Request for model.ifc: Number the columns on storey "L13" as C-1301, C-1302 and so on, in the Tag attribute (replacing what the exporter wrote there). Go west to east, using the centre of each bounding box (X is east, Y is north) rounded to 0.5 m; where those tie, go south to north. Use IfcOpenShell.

First a look at what the model holds.

```python
import ifcopenshell
import ifcopenshell.util.element
import ifcopenshell.util.placement

model = ifcopenshell.open("model.ifc")
print(model.schema)
storey = next(s for s in model.by_type("IfcBuildingStorey") if s.Name == "L13")
columns = [e for e in ifcopenshell.util.element.get_decomposition(storey) if e.is_a("IfcColumn")]
for e in sorted(columns, key=lambda e: e.id()):
    origin = ifcopenshell.util.placement.get_local_placement(e.ObjectPlacement)[:3, 3]
    print(e.id(), e.Tag, e.Name, origin.round(2) + 0.0, sep=" | ")
```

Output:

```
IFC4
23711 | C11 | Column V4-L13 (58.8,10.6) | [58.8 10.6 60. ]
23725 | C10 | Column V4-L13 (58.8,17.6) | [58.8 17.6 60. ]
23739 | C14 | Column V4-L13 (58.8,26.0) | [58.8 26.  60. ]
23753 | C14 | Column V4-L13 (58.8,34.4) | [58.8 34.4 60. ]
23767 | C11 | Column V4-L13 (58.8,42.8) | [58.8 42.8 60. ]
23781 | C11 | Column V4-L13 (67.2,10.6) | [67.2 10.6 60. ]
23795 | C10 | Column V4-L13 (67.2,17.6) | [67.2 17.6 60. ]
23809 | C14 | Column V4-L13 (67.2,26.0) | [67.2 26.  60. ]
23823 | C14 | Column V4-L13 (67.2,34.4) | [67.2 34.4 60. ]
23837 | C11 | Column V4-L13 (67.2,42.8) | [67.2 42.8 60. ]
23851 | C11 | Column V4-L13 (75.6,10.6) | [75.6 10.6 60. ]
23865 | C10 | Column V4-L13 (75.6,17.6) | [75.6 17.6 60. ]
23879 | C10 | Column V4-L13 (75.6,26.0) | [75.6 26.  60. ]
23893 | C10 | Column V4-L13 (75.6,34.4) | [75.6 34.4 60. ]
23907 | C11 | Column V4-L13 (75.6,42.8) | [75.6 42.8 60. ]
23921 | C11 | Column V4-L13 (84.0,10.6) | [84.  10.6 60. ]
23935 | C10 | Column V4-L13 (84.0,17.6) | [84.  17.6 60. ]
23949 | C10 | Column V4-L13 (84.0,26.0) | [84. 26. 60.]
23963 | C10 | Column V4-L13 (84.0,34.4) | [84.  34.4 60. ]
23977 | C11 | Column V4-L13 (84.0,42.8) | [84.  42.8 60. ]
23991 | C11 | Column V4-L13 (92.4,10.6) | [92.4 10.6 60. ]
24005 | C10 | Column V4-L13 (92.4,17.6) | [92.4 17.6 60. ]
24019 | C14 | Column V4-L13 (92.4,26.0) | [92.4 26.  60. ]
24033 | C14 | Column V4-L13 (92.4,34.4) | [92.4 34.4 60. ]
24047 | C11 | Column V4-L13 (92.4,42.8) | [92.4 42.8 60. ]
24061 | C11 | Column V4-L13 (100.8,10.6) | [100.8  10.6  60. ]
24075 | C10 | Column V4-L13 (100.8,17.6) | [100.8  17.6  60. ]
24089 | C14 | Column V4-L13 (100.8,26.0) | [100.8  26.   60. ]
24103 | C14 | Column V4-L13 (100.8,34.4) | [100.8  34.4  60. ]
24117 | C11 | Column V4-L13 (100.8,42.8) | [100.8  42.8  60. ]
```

```python
import ifcopenshell
import ifcopenshell.geom
import ifcopenshell.util.element
import ifcopenshell.util.shape

model = ifcopenshell.open("model.ifc")
settings = ifcopenshell.geom.settings()
settings.set("use-world-coords", True)


def centre(element):
    shape = ifcopenshell.geom.create_shape(settings, element)
    return ifcopenshell.util.shape.get_bbox_centroid(shape.geometry)


storey = next(s for s in model.by_type("IfcBuildingStorey") if s.Name == "L13")
columns = [e for e in ifcopenshell.util.element.get_decomposition(storey) if e.is_a("IfcColumn")]

# Insertion points can sit at a corner or the storey origin, so sort by the geometry (in metres).
centres = {e: centre(e) for e in columns}
columns.sort(key=lambda e: (round(centres[e][0] / 0.5), centres[e][1]))

for i, e in enumerate(columns, start=1):
    number = f"C-13{i:02d}"
    e.Tag = number
    print(e.id(), number)

model.write("model_edited.ifc")
```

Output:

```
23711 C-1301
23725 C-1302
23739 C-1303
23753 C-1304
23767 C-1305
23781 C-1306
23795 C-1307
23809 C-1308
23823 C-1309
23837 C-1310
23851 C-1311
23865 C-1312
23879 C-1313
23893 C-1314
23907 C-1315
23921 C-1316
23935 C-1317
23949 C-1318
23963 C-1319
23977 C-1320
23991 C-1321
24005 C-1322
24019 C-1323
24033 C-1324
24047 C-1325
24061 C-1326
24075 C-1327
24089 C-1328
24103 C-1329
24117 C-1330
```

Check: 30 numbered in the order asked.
